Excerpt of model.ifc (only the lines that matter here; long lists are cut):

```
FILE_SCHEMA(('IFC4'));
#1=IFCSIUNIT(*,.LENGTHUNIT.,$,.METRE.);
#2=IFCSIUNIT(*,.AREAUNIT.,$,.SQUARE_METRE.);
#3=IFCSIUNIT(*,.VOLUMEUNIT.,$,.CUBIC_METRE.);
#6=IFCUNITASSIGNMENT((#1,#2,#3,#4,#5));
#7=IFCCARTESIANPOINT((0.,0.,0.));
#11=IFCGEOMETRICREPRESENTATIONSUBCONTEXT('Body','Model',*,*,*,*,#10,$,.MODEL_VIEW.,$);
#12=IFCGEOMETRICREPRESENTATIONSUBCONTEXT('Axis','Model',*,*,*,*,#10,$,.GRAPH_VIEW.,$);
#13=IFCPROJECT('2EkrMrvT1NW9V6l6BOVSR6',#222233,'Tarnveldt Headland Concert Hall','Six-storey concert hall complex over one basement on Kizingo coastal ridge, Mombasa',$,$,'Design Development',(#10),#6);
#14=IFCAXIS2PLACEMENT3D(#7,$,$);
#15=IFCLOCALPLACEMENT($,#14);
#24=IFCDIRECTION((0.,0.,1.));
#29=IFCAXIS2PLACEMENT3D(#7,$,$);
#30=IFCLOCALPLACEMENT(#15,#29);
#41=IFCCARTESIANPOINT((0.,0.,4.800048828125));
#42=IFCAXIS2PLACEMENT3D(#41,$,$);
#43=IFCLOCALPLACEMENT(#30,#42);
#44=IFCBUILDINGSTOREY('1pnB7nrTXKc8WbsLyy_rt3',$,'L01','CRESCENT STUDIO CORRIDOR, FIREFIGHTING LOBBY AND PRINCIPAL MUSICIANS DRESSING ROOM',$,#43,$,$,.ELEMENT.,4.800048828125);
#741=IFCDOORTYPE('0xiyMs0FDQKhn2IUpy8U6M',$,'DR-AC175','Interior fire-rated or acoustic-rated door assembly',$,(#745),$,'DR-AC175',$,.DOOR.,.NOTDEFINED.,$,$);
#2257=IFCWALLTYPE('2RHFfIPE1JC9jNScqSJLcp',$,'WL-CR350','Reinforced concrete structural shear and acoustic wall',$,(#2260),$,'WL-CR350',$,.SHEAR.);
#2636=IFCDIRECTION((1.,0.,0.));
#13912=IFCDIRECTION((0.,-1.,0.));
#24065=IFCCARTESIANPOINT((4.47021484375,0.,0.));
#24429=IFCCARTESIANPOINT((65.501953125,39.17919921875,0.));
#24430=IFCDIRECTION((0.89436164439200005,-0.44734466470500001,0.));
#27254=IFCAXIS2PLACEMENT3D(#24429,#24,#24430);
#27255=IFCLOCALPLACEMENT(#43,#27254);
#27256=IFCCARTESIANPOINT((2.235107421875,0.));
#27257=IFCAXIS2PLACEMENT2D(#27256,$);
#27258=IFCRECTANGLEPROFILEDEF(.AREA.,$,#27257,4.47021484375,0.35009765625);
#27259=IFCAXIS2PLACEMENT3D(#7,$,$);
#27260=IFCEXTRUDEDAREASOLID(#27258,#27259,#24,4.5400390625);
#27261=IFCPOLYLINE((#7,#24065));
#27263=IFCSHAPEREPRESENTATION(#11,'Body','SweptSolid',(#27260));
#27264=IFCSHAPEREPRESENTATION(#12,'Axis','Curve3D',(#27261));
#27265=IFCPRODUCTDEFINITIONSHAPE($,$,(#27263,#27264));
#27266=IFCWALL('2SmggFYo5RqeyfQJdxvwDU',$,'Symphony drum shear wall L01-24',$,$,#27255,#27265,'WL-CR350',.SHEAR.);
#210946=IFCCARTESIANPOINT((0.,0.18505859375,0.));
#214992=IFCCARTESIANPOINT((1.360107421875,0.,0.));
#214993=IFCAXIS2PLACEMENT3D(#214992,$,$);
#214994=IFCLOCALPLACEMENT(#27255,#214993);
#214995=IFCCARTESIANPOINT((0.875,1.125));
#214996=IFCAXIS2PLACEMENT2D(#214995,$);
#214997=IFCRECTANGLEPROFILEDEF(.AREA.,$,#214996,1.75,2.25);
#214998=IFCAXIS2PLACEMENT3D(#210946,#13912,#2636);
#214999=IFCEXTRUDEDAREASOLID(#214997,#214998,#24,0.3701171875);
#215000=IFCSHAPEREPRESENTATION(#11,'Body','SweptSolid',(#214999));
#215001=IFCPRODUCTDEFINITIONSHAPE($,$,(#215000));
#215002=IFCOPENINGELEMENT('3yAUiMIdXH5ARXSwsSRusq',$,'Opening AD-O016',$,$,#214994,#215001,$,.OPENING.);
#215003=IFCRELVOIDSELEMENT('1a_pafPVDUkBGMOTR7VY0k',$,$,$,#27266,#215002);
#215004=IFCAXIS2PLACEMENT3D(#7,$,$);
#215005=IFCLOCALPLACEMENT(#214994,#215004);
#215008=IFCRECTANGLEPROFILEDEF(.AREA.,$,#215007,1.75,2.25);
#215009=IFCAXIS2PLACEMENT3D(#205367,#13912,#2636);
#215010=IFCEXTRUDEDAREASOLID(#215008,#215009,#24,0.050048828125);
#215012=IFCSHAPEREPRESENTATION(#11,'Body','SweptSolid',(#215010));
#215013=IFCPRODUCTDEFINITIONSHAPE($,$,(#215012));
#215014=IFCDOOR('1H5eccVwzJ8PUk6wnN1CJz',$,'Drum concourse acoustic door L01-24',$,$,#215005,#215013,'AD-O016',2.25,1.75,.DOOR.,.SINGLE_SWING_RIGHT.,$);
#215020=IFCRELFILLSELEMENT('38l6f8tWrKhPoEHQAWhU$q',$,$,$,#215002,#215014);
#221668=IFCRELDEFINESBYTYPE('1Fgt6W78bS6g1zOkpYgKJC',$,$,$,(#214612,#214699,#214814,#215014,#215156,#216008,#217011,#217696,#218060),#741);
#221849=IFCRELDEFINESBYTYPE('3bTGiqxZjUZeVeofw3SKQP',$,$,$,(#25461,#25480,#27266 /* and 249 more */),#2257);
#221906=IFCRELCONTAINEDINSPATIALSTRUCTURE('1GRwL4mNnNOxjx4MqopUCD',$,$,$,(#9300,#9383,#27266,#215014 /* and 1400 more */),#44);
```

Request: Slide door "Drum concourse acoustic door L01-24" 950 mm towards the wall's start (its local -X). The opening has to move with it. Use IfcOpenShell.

```python
import ifcopenshell
import ifcopenshell.api.geometry
import ifcopenshell.util.placement
import ifcopenshell.util.unit

model = ifcopenshell.open("model.ifc")
unit_scale = ifcopenshell.util.unit.calculate_unit_scale(model)

door = model.by_guid("1H5eccVwzJ8PUk6wnN1CJz")
opening = door.FillsVoids[0].RelatingOpeningElement
wall = opening.VoidsElements[0].RelatingBuildingElement

wall_matrix = ifcopenshell.util.placement.get_local_placement(wall.ObjectPlacement)
shift = wall_matrix[:3, 0] * -0.95 / unit_scale
before = ifcopenshell.util.placement.get_local_placement(door.ObjectPlacement)[:3, 3].copy()

# The door is placed relative to its opening, so it follows when the opening moves.
matrix = ifcopenshell.util.placement.get_local_placement(opening.ObjectPlacement)
matrix[:3, 3] += shift
ifcopenshell.api.geometry.edit_object_placement(
    model, product=opening, matrix=matrix, is_si=False, should_transform_children=True
)

after = ifcopenshell.util.placement.get_local_placement(door.ObjectPlacement)[:3, 3]
print("door moved by", (after - before).round(3) + 0.0)

model.write("model_updated.ifc")
```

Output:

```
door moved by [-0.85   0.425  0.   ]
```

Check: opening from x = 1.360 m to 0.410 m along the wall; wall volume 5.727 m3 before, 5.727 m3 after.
